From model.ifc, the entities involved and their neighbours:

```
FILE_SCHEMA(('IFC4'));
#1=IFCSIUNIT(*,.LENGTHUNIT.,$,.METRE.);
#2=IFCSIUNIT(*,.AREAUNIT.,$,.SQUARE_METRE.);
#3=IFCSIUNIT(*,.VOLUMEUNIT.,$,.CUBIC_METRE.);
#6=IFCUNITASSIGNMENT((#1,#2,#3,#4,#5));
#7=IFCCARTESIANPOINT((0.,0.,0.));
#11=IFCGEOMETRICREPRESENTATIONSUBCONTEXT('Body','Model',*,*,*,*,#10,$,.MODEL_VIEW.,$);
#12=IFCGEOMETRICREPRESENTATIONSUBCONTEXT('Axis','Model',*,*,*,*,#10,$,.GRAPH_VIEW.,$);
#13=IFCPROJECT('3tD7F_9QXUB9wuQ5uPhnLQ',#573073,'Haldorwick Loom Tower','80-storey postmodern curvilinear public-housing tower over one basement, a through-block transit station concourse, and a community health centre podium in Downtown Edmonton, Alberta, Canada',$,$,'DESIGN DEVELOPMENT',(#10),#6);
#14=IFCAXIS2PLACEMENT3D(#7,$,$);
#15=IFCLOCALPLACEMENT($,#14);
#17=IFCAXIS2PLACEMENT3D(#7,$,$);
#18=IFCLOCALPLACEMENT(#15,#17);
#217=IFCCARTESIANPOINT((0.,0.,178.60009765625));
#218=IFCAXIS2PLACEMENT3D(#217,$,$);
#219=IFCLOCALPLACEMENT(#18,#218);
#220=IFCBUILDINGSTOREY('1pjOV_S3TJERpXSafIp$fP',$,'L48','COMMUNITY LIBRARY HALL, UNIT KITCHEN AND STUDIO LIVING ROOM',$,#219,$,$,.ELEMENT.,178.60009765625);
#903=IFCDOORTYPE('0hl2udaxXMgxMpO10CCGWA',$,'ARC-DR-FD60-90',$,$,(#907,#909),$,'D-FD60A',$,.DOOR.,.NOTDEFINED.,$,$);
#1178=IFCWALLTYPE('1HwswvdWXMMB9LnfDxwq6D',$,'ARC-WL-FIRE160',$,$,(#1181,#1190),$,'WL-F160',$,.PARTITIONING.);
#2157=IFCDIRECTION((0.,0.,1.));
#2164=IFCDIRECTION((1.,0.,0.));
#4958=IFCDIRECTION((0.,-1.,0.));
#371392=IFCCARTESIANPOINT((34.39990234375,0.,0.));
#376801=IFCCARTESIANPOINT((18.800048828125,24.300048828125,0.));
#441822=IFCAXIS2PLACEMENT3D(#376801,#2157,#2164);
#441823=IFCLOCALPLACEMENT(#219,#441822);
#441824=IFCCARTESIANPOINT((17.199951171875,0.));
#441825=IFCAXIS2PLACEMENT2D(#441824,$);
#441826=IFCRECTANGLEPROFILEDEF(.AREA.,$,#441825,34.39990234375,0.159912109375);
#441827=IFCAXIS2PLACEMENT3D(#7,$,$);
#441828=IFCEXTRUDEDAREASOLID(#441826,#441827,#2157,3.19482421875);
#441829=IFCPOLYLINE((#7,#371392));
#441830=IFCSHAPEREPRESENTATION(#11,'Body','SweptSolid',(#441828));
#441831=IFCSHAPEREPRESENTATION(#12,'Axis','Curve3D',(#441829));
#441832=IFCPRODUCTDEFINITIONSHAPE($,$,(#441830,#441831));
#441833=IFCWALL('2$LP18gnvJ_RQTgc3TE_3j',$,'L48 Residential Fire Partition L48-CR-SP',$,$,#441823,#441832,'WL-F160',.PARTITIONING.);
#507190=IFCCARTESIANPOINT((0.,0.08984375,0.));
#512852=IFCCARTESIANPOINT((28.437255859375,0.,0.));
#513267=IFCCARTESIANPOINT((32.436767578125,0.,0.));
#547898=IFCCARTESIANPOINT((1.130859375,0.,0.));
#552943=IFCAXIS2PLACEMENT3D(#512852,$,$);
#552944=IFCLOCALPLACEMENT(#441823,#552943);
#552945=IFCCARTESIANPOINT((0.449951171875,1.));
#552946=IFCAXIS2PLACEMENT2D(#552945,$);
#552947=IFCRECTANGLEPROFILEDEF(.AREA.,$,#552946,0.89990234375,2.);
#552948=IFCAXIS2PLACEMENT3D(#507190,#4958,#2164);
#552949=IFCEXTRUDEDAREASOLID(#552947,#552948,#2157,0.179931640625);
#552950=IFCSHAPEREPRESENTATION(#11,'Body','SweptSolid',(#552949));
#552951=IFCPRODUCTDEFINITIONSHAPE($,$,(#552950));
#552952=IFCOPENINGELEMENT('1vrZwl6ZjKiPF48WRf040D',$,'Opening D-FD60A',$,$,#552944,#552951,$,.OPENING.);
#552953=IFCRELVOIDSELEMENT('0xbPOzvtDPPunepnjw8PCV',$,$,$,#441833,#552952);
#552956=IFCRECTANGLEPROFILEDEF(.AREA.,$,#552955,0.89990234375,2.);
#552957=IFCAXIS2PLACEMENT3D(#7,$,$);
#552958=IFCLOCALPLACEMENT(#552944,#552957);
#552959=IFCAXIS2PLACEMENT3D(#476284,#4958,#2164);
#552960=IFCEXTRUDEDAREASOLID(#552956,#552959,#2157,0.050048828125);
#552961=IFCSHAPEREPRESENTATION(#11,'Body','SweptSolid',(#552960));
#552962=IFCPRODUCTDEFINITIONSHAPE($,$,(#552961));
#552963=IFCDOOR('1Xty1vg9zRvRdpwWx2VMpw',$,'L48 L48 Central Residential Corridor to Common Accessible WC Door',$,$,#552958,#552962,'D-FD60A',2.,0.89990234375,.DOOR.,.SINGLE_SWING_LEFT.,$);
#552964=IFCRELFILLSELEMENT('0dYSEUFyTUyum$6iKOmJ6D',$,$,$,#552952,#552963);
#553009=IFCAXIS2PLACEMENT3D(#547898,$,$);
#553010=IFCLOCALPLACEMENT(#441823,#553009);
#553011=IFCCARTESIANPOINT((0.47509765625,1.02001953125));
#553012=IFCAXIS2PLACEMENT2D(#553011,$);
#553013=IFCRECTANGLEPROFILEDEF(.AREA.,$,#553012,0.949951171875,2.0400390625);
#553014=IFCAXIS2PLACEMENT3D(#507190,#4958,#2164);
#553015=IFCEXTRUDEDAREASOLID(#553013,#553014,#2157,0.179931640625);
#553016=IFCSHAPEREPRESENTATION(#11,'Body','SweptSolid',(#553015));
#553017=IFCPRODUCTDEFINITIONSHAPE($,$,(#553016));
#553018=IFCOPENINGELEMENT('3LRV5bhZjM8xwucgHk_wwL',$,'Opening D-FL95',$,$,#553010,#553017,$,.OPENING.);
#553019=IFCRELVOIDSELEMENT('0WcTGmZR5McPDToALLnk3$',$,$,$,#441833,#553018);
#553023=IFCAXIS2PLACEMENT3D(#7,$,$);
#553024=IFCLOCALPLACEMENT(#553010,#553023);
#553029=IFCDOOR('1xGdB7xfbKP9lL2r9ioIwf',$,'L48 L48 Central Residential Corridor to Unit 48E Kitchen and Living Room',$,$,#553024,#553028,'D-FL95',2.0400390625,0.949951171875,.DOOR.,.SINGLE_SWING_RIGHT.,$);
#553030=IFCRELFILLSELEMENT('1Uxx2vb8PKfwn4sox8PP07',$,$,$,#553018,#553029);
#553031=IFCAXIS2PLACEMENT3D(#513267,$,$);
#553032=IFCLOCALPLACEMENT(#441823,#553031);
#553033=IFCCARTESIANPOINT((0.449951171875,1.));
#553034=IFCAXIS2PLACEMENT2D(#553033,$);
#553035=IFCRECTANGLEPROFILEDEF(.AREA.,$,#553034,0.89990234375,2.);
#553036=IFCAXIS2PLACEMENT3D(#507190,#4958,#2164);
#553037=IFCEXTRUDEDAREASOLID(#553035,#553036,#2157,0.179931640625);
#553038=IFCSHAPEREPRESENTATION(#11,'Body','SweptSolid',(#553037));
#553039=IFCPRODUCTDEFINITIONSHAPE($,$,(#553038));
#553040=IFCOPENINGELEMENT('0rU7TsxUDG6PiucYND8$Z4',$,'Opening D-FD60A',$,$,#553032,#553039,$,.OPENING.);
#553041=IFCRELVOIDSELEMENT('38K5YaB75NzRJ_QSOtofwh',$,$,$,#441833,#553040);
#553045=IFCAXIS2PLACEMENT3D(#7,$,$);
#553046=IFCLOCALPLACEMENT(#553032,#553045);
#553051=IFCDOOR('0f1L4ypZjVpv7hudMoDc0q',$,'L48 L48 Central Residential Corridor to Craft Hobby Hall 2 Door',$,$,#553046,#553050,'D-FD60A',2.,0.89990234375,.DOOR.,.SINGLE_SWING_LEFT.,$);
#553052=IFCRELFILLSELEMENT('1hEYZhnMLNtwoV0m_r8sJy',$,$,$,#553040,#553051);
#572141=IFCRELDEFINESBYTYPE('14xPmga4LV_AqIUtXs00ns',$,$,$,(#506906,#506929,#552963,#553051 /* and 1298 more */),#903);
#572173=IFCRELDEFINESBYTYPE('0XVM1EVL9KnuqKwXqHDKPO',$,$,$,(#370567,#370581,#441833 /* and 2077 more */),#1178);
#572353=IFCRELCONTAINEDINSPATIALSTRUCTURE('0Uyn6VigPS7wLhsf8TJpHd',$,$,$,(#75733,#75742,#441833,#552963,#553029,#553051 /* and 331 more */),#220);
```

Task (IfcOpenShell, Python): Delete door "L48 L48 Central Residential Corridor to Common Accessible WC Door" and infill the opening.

```python
import ifcopenshell
import ifcopenshell.api.feature
import ifcopenshell.api.root
import ifcopenshell.geom
import ifcopenshell.util.shape

model = ifcopenshell.open("model.ifc")
settings = ifcopenshell.geom.settings()


def volume(element):
    """Net volume in cubic metres, openings subtracted."""
    shape = ifcopenshell.geom.create_shape(settings, element)
    return ifcopenshell.util.shape.get_volume(shape.geometry)


door = model.by_guid("1Xty1vg9zRvRdpwWx2VMpw")
opening = door.FillsVoids[0].RelatingOpeningElement
wall = opening.VoidsElements[0].RelatingBuildingElement
before = volume(wall)

ifcopenshell.api.root.remove_product(model, product=door)
ifcopenshell.api.feature.remove_feature(model, feature=opening)

after = volume(wall)

print(f"wall volume {before:.3f} -> {after:.3f} m3")

model.write("model-out.ifc")
```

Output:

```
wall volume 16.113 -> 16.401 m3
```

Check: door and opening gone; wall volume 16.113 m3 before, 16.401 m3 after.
